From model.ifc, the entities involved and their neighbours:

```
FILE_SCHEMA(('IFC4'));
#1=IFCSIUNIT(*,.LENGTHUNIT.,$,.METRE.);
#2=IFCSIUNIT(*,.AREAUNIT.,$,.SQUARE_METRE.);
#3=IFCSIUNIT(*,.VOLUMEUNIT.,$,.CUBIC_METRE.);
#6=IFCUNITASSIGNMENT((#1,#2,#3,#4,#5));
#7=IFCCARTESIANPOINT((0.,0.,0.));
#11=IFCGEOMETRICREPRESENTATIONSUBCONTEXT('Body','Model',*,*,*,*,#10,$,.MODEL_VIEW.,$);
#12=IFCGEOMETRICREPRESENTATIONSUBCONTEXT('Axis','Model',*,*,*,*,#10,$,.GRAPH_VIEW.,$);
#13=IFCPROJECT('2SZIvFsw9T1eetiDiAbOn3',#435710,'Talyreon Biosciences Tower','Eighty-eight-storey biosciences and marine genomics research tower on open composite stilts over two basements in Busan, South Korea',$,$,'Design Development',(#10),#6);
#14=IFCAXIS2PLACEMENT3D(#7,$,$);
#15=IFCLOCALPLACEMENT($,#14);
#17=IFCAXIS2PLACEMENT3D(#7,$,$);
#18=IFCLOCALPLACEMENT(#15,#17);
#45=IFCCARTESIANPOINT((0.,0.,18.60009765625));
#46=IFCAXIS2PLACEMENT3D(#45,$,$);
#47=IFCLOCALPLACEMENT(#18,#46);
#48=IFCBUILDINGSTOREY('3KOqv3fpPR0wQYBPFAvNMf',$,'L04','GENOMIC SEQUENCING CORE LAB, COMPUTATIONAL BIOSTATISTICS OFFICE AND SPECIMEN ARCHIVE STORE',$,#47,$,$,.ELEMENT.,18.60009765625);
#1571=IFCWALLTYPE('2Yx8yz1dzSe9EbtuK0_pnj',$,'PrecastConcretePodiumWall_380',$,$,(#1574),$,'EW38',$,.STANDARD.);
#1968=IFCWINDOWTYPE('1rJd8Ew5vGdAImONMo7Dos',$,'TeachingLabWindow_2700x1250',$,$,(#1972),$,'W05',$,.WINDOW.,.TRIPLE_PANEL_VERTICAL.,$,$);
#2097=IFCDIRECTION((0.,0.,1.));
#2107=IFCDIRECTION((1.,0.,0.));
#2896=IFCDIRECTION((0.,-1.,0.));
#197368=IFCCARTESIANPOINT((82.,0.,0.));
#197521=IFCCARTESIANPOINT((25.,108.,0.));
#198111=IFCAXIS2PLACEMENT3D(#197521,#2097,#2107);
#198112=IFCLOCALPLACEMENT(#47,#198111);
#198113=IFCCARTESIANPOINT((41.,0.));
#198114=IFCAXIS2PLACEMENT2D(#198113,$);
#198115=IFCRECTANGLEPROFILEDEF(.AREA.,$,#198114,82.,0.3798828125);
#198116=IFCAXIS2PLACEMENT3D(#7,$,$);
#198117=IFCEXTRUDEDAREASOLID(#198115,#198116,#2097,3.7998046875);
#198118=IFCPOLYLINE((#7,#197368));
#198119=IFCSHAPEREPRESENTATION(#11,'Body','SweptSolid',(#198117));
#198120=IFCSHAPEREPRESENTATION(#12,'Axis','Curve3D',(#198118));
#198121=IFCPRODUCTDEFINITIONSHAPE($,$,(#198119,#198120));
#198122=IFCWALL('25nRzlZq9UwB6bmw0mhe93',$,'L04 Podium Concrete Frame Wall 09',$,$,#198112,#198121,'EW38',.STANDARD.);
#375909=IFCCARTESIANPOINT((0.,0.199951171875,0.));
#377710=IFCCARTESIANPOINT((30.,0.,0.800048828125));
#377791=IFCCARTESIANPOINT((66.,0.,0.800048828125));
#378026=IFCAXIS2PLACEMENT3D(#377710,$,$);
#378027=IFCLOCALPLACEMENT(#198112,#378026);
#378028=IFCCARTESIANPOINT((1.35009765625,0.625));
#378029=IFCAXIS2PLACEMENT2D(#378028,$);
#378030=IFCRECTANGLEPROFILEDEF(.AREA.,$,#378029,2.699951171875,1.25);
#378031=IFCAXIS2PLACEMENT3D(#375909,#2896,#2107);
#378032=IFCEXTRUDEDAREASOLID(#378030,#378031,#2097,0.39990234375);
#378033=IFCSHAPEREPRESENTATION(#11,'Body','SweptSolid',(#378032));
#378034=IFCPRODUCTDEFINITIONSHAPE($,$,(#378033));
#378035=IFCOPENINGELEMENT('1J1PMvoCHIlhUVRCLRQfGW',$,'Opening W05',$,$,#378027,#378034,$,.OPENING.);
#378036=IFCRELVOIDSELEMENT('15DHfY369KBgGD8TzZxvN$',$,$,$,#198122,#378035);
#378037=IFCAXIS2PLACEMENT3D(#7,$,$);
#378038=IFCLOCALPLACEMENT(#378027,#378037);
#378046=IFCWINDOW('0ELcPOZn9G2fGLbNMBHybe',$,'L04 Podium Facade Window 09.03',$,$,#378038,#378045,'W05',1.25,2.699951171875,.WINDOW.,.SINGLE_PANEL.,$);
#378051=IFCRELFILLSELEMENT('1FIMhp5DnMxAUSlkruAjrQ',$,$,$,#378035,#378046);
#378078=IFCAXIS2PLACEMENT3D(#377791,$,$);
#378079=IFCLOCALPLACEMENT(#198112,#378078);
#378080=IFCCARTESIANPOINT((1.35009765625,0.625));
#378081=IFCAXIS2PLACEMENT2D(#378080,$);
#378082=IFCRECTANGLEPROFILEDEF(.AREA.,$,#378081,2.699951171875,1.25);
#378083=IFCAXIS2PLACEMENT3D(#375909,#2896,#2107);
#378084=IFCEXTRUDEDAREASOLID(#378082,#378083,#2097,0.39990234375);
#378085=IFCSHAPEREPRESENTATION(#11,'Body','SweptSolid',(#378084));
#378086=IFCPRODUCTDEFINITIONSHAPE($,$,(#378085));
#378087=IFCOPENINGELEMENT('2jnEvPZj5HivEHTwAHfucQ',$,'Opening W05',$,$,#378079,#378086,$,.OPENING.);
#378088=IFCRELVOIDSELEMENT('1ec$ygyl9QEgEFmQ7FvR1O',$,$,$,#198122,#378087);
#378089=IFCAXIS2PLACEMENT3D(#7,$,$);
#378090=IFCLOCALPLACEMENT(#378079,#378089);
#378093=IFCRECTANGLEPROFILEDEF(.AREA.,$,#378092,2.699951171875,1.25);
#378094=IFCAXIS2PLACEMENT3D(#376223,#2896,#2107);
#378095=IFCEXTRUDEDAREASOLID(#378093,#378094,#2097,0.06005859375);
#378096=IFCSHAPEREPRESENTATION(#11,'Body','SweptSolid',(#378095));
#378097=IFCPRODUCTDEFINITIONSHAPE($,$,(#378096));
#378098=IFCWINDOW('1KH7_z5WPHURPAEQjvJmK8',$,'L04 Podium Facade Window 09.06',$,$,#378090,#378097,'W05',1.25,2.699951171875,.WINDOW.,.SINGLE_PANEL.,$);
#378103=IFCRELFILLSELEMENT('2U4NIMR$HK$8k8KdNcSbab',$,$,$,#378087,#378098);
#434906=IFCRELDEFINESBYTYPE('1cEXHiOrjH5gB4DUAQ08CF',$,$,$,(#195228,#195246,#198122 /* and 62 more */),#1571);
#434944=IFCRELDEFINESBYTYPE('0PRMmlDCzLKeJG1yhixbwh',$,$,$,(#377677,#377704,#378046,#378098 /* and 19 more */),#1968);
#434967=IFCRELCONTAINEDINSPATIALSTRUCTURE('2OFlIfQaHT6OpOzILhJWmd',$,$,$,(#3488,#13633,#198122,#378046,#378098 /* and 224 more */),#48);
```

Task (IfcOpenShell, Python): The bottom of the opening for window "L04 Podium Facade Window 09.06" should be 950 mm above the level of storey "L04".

```python
import numpy as np
import ifcopenshell
import ifcopenshell.api.geometry
import ifcopenshell.geom
import ifcopenshell.util.element
import ifcopenshell.util.placement
import ifcopenshell.util.shape
import ifcopenshell.util.unit

model = ifcopenshell.open("model.ifc")
unit_scale = ifcopenshell.util.unit.calculate_unit_scale(model)

window = model.by_guid("1KH7_z5WPHURPAEQjvJmK8")
opening = window.FillsVoids[0].RelatingOpeningElement
storey = ifcopenshell.util.element.get_container(window, ifc_class="IfcBuildingStorey")
level = ifcopenshell.util.placement.get_local_placement(storey.ObjectPlacement)[2, 3]

# The opening's origin need not be at the sill, so measure its lowest point.
shape = ifcopenshell.geom.create_shape(ifcopenshell.geom.settings(), opening)
bottom = ifcopenshell.util.shape.get_shape_bottom_elevation(shape, shape.geometry) / unit_scale
dz = level + 0.95 / unit_scale - bottom

shift = np.array([0.0, 0.0, dz])
# The window is placed relative to its opening, so it follows when the opening moves.
matrix = ifcopenshell.util.placement.get_local_placement(opening.ObjectPlacement)
matrix[:3, 3] += shift
ifcopenshell.api.geometry.edit_object_placement(
    model, product=opening, matrix=matrix, is_si=False, should_transform_children=True
)

print(f"moved by {dz * unit_scale:+.3f} m")

model.write("model-out.ifc")
```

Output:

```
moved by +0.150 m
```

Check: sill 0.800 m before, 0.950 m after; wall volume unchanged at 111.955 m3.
